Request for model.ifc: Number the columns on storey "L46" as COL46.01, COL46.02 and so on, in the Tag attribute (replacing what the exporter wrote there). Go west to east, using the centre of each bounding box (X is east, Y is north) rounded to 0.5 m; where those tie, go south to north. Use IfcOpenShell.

First a look at what the model holds.

```python
import ifcopenshell
import ifcopenshell.util.element
import ifcopenshell.util.placement

model = ifcopenshell.open("model.ifc")
print(model.schema)
storey = next(s for s in model.by_type("IfcBuildingStorey") if s.Name == "L46")
columns = [e for e in ifcopenshell.util.element.get_decomposition(storey) if e.is_a("IfcColumn")]
for e in sorted(columns, key=lambda e: e.id()):
    origin = ifcopenshell.util.placement.get_local_placement(e.ObjectPlacement)[:3, 3]
    print(e.id(), e.Tag, e.Name, origin.round(2) + 0.0, sep=" | ")
```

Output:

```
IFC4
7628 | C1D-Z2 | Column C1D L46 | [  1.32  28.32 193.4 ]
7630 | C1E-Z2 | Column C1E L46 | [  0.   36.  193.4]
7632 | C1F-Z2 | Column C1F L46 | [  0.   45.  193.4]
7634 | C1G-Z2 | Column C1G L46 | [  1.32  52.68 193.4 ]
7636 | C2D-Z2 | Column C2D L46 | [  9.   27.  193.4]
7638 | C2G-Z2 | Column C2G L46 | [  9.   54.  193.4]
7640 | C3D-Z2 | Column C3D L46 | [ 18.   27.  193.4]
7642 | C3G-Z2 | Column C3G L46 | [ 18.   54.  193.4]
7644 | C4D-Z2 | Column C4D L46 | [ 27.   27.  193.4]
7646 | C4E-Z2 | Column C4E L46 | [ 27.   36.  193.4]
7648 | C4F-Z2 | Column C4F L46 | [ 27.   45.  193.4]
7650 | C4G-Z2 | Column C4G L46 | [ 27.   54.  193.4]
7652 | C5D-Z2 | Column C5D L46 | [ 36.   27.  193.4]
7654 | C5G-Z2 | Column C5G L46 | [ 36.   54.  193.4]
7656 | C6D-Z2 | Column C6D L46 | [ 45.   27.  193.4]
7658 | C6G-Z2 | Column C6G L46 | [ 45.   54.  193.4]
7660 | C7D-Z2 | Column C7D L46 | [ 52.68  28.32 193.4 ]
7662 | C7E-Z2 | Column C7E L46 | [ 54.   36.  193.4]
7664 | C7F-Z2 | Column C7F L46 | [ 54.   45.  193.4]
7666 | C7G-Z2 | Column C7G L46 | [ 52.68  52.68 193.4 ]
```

```python
import ifcopenshell
import ifcopenshell.geom
import ifcopenshell.util.element
import ifcopenshell.util.shape

model = ifcopenshell.open("model.ifc")
settings = ifcopenshell.geom.settings()
settings.set("use-world-coords", True)


def centre(element):
    shape = ifcopenshell.geom.create_shape(settings, element)
    return ifcopenshell.util.shape.get_bbox_centroid(shape.geometry)


storey = next(s for s in model.by_type("IfcBuildingStorey") if s.Name == "L46")
columns = [e for e in ifcopenshell.util.element.get_decomposition(storey) if e.is_a("IfcColumn")]

# Insertion points can sit at a corner or the storey origin, so sort by the geometry (in metres).
centres = {e: centre(e) for e in columns}
columns.sort(key=lambda e: (round(centres[e][0] / 0.5), centres[e][1]))

for i, e in enumerate(columns, start=1):
    number = f"COL46.{i:02d}"
    e.Tag = number
    print(e.id(), number)

model.write("model_rev.ifc")
```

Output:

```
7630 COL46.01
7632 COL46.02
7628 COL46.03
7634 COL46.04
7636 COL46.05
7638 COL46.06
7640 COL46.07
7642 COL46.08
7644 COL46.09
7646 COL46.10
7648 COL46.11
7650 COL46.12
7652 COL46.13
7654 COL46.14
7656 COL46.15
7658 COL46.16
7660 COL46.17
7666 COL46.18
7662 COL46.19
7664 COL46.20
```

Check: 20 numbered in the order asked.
